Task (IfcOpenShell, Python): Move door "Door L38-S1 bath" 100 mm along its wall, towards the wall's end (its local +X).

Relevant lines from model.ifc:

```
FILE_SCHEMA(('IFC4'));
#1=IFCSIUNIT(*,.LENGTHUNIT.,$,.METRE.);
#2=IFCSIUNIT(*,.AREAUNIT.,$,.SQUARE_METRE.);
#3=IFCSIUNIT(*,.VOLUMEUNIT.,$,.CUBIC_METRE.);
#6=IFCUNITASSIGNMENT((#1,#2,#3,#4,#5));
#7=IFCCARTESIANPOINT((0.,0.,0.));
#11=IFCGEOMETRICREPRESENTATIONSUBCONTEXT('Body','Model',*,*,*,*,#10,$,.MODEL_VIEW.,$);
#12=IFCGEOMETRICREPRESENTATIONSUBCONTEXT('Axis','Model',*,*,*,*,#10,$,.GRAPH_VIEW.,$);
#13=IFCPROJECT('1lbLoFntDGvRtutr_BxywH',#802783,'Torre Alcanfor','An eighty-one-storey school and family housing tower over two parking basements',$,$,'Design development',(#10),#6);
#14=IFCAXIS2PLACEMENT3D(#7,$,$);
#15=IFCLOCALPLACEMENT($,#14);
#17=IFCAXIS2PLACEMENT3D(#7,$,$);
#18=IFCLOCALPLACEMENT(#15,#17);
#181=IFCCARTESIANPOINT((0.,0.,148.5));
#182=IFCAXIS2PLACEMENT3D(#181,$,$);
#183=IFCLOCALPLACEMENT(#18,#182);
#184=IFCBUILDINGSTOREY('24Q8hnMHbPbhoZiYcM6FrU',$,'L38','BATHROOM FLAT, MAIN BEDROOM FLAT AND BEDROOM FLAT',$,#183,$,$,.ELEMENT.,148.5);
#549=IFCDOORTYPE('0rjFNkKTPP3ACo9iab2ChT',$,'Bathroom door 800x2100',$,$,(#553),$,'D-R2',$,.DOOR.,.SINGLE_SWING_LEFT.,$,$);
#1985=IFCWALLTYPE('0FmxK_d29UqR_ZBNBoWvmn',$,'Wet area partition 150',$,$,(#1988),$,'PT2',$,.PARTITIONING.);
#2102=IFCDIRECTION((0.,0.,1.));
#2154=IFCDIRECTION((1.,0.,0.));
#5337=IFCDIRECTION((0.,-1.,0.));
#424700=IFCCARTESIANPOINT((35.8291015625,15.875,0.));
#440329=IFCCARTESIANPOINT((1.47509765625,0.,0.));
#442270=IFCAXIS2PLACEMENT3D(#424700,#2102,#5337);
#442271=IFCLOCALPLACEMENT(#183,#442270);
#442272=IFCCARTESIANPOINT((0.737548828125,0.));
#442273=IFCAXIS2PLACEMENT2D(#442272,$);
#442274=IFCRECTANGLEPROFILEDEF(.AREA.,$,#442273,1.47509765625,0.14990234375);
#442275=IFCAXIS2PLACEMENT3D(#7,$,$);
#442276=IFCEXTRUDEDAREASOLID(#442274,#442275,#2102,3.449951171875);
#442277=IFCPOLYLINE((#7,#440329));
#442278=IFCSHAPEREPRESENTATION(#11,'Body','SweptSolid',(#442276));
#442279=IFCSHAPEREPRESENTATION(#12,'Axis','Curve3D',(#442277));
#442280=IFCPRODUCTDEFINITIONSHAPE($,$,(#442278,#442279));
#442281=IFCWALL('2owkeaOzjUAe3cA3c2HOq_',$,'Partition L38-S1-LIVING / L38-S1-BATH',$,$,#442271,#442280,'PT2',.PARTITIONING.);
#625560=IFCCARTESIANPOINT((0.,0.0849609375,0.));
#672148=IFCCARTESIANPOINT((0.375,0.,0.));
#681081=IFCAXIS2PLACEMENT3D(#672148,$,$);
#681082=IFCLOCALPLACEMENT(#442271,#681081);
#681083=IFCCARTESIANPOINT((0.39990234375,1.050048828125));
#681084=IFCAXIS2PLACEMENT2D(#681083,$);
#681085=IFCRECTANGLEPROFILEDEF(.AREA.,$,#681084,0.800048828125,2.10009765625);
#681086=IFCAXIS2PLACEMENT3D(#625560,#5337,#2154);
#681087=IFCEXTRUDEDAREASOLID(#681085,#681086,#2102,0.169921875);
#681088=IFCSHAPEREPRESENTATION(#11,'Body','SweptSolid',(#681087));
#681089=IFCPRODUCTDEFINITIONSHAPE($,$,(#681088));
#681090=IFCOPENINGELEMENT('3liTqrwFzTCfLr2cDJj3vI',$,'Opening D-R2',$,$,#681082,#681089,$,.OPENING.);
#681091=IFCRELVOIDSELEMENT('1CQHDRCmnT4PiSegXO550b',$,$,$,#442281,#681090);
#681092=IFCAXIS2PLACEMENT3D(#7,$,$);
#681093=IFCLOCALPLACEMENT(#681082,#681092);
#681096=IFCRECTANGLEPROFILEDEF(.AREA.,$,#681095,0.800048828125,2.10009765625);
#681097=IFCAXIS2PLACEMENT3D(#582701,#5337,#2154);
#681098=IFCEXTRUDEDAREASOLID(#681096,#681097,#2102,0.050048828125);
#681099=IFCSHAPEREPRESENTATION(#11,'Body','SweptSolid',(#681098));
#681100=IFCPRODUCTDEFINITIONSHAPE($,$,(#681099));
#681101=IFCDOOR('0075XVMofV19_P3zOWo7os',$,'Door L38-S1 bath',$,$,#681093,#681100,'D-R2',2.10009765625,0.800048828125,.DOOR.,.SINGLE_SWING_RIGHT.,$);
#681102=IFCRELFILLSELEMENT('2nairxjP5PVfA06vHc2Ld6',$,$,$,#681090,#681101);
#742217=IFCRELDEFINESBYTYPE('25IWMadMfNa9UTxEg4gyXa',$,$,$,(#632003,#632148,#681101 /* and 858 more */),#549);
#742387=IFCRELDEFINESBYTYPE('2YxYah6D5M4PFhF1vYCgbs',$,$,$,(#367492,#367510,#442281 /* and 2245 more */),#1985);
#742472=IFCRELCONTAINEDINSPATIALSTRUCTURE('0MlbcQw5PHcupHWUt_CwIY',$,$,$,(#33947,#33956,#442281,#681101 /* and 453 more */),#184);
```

```python
import ifcopenshell
import ifcopenshell.api.geometry
import ifcopenshell.util.placement
import ifcopenshell.util.unit

model = ifcopenshell.open("model.ifc")
unit_scale = ifcopenshell.util.unit.calculate_unit_scale(model)

door = model.by_guid("0075XVMofV19_P3zOWo7os")
opening = door.FillsVoids[0].RelatingOpeningElement
wall = opening.VoidsElements[0].RelatingBuildingElement

wall_matrix = ifcopenshell.util.placement.get_local_placement(wall.ObjectPlacement)
shift = wall_matrix[:3, 0] * 0.1 / unit_scale
before = ifcopenshell.util.placement.get_local_placement(door.ObjectPlacement)[:3, 3].copy()

# The door is placed relative to its opening, so it follows when the opening moves.
matrix = ifcopenshell.util.placement.get_local_placement(opening.ObjectPlacement)
matrix[:3, 3] += shift
ifcopenshell.api.geometry.edit_object_placement(
    model, product=opening, matrix=matrix, is_si=False, should_transform_children=True
)

after = ifcopenshell.util.placement.get_local_placement(door.ObjectPlacement)[:3, 3]
print("door moved by", (after - before).round(3) + 0.0)

model.write("model_rev.ifc")
```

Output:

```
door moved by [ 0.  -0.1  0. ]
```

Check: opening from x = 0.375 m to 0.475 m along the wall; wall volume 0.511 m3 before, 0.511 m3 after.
